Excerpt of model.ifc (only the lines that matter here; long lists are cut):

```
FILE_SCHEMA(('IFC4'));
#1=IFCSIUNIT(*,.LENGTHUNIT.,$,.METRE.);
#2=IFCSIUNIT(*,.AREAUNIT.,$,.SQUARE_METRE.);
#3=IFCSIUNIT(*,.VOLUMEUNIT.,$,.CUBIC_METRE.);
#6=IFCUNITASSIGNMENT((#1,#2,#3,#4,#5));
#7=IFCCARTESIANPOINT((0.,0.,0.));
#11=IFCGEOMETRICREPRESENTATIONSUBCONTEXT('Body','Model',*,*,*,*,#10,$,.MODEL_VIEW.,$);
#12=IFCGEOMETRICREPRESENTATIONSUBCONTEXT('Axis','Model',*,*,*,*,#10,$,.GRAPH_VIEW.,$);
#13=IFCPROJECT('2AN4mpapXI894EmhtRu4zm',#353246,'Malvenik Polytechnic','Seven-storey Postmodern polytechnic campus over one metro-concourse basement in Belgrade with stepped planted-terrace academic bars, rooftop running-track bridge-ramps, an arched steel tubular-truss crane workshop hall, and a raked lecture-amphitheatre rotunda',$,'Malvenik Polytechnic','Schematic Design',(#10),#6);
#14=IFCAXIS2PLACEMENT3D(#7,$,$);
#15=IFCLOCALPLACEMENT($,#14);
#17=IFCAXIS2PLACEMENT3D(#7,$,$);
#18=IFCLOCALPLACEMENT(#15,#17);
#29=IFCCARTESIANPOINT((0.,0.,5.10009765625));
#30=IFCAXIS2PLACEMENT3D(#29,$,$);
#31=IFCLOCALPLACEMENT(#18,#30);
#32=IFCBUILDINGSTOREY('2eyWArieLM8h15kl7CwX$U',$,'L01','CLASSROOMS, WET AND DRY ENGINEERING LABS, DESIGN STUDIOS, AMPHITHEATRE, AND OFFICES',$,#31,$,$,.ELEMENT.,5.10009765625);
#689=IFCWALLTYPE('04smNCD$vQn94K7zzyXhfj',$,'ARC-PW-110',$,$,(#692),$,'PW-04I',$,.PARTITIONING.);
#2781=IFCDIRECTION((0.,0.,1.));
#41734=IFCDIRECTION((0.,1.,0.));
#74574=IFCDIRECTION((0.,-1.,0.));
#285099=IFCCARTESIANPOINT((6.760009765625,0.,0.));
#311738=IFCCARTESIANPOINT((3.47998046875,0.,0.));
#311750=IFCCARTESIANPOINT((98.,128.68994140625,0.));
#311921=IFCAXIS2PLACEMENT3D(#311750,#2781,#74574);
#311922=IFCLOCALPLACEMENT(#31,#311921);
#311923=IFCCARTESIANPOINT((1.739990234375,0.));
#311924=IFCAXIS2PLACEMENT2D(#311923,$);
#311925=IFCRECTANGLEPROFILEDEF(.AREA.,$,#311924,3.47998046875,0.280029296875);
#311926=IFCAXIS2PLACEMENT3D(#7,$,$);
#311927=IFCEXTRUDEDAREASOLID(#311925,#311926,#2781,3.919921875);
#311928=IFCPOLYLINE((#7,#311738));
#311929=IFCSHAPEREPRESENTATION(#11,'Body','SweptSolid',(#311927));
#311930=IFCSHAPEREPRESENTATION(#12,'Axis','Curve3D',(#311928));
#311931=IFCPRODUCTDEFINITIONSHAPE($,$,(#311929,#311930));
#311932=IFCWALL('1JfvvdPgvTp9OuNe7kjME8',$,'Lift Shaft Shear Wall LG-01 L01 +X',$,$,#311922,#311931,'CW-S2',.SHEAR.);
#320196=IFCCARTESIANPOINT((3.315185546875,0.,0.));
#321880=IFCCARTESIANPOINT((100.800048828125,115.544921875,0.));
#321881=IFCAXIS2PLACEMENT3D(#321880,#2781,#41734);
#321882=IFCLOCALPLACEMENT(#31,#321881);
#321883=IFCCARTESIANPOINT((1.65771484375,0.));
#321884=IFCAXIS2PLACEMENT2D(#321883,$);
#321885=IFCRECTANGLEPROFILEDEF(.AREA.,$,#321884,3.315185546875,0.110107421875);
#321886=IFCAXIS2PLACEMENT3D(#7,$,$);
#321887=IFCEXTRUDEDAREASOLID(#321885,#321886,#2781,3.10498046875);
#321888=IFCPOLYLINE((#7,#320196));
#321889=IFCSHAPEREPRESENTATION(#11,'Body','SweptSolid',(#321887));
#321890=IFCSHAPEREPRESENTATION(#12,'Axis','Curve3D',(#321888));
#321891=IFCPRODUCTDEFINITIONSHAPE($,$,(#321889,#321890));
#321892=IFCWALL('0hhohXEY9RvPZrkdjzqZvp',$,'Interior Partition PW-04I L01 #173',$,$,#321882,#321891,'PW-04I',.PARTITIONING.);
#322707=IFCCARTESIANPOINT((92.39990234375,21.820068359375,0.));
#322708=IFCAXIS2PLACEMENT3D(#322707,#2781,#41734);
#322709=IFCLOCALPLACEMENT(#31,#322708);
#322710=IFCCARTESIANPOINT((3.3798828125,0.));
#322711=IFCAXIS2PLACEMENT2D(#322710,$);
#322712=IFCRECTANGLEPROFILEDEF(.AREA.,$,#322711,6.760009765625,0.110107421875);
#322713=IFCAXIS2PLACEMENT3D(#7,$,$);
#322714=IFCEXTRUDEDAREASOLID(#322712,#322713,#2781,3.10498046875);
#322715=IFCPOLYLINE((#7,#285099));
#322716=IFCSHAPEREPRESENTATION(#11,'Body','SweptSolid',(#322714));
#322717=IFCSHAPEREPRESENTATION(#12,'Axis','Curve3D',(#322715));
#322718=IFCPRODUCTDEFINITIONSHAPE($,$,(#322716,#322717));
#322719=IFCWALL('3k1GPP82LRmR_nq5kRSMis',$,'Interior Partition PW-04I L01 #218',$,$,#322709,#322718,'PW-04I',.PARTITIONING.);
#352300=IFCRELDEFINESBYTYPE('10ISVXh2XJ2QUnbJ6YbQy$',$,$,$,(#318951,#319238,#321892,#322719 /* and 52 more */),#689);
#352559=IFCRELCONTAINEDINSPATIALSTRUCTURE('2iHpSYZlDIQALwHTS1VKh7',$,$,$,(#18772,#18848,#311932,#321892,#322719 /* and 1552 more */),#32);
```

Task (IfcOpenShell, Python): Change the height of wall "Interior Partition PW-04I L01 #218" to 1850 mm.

```python
import ifcopenshell
import ifcopenshell.geom
import ifcopenshell.util.representation
import ifcopenshell.util.shape

model = ifcopenshell.open("model.ifc")
settings = ifcopenshell.geom.settings()


def volume(element):
    """Net volume in cubic metres, openings subtracted."""
    shape = ifcopenshell.geom.create_shape(settings, element)
    return ifcopenshell.util.shape.get_volume(shape.geometry)


wall = model.by_guid("3k1GPP82LRmR_nq5kRSMis")
before = volume(wall)

body = ifcopenshell.util.representation.get_representation(wall, "Model", "Body")
solid = body.Items[0]
old_height = solid.Depth
solid.Depth = 1.85
after = volume(wall)

print(f"height {old_height:g} -> {solid.Depth:g}, volume {before:.3f} -> {after:.3f} m3")

model.write("model_v2.ifc")
```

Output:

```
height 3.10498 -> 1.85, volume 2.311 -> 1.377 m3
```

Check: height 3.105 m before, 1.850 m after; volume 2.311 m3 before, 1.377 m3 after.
